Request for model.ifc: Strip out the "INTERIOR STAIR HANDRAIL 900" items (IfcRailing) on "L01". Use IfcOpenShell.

First a look at what the model holds.

```python
import ifcopenshell
import ifcopenshell.util.element

model = ifcopenshell.open("model.ifc")
print(model.schema)
storey = next(s for s in model.by_type("IfcBuildingStorey") if s.Name == "L01")
railings = [e for e in ifcopenshell.util.element.get_decomposition(storey) if e.is_a("IfcRailing")]
seen = {}
for e in railings:
    element_type = ifcopenshell.util.element.get_type(e)
    name = element_type.Name if element_type not in (None, e) else None
    seen[name] = seen.get(name, 0) + 1
for name, count in sorted(seen.items(), key=str):
    print(count, "x", name)
```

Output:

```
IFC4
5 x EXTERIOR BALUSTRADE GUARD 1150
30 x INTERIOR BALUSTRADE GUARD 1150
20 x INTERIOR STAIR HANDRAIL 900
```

```python
import ifcopenshell
import ifcopenshell.api.root
import ifcopenshell.util.element

model = ifcopenshell.open("model.ifc")

storey = next(s for s in model.by_type("IfcBuildingStorey") if s.Name == "L01")
railings = [e for e in ifcopenshell.util.element.get_decomposition(storey) if e.is_a("IfcRailing")]
targets = [e for e in railings if (t := ifcopenshell.util.element.get_type(e)) not in (None, e) and t.Name == "INTERIOR STAIR HANDRAIL 900"]

for e in targets:
    ifcopenshell.api.root.remove_product(model, product=e)
print(len(targets), "removed")

model.write("model_v2.ifc")
```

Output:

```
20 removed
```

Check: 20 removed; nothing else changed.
